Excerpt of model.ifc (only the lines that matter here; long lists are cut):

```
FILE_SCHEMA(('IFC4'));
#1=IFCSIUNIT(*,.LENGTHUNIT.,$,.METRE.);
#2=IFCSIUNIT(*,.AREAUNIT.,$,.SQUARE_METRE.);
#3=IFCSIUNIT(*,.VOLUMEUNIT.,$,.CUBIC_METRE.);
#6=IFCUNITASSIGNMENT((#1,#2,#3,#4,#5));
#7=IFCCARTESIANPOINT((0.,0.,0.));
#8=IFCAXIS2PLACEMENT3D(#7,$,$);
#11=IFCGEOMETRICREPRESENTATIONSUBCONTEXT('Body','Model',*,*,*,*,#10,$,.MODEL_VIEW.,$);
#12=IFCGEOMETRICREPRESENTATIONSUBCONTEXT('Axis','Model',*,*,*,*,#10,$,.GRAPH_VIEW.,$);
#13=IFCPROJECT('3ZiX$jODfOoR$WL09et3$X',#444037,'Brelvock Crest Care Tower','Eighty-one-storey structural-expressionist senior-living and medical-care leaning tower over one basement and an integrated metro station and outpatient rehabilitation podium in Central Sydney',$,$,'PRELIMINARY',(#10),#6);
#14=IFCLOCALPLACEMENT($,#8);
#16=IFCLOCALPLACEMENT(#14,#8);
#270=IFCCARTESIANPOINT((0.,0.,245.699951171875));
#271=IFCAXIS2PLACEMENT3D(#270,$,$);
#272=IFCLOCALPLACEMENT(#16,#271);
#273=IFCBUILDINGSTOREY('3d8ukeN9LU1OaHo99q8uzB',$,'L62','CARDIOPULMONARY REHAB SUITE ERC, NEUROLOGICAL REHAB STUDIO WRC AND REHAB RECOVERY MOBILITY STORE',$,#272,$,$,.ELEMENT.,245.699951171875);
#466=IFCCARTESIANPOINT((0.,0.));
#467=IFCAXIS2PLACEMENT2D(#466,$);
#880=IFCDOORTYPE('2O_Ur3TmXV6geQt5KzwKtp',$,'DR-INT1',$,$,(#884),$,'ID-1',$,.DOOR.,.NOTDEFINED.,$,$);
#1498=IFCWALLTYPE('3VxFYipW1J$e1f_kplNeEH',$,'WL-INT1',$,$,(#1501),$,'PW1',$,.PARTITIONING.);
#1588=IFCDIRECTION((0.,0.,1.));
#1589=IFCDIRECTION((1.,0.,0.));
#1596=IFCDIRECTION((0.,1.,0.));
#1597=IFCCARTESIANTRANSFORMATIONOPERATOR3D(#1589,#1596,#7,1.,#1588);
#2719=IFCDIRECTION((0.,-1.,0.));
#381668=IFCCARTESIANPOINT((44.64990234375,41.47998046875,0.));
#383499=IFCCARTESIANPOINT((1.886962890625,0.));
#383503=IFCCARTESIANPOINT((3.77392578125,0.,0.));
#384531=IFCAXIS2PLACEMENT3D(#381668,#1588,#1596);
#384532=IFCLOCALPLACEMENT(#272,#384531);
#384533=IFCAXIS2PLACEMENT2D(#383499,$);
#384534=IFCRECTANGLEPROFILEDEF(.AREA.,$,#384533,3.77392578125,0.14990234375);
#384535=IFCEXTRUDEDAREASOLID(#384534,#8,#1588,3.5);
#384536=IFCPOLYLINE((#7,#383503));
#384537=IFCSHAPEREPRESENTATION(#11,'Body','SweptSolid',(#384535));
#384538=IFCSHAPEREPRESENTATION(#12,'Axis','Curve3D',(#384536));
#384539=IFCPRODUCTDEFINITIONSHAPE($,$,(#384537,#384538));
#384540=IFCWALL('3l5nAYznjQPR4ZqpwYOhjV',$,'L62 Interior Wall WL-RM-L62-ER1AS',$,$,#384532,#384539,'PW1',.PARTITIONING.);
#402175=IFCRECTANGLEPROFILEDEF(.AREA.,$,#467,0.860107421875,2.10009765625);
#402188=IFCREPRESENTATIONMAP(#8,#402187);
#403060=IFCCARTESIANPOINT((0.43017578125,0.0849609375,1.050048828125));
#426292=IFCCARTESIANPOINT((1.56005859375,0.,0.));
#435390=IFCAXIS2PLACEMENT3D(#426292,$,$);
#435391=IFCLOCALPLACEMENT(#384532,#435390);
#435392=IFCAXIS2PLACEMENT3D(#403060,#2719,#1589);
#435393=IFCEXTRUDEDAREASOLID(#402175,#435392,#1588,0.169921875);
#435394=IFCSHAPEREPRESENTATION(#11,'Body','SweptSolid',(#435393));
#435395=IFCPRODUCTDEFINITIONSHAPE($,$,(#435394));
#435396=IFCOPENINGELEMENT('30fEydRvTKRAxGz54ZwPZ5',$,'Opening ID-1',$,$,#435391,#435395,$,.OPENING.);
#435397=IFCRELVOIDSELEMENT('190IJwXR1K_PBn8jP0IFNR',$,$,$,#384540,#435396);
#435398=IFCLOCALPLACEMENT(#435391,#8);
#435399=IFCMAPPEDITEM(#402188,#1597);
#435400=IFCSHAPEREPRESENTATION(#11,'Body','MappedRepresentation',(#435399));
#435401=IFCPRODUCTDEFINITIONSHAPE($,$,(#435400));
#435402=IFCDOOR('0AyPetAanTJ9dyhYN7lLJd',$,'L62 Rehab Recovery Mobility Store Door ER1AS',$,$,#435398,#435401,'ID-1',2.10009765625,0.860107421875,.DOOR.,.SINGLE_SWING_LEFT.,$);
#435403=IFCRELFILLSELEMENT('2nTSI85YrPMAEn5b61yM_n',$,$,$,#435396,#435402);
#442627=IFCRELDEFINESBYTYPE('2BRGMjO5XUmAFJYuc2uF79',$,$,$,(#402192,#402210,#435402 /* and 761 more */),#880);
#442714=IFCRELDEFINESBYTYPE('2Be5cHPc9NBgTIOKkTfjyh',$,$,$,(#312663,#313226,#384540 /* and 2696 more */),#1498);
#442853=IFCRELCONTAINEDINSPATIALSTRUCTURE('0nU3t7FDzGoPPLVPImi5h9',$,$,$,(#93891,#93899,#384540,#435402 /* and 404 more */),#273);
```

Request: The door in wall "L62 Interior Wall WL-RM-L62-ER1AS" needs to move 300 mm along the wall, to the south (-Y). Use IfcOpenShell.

```python
import ifcopenshell
import ifcopenshell.api.geometry
import ifcopenshell.util.placement

model = ifcopenshell.open("model.ifc")

door = model.by_id(435402)
opening = door.FillsVoids[0].RelatingOpeningElement
wall = opening.VoidsElements[0].RelatingBuildingElement

wall_matrix = ifcopenshell.util.placement.get_local_placement(wall.ObjectPlacement)
shift = wall_matrix[:3, 0] * -0.3
before = ifcopenshell.util.placement.get_local_placement(door.ObjectPlacement)[:3, 3].copy()

# The door is placed relative to its opening, so it follows when the opening moves.
matrix = ifcopenshell.util.placement.get_local_placement(opening.ObjectPlacement)
matrix[:3, 3] += shift
ifcopenshell.api.geometry.edit_object_placement(
    model, product=opening, matrix=matrix, is_si=False, should_transform_children=True
)

after = ifcopenshell.util.placement.get_local_placement(door.ObjectPlacement)[:3, 3]
print("door moved by", (after - before).round(3) + 0.0)

model.write("model_edited.ifc")
```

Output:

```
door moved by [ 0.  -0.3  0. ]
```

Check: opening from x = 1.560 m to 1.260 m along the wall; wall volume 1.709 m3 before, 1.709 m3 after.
